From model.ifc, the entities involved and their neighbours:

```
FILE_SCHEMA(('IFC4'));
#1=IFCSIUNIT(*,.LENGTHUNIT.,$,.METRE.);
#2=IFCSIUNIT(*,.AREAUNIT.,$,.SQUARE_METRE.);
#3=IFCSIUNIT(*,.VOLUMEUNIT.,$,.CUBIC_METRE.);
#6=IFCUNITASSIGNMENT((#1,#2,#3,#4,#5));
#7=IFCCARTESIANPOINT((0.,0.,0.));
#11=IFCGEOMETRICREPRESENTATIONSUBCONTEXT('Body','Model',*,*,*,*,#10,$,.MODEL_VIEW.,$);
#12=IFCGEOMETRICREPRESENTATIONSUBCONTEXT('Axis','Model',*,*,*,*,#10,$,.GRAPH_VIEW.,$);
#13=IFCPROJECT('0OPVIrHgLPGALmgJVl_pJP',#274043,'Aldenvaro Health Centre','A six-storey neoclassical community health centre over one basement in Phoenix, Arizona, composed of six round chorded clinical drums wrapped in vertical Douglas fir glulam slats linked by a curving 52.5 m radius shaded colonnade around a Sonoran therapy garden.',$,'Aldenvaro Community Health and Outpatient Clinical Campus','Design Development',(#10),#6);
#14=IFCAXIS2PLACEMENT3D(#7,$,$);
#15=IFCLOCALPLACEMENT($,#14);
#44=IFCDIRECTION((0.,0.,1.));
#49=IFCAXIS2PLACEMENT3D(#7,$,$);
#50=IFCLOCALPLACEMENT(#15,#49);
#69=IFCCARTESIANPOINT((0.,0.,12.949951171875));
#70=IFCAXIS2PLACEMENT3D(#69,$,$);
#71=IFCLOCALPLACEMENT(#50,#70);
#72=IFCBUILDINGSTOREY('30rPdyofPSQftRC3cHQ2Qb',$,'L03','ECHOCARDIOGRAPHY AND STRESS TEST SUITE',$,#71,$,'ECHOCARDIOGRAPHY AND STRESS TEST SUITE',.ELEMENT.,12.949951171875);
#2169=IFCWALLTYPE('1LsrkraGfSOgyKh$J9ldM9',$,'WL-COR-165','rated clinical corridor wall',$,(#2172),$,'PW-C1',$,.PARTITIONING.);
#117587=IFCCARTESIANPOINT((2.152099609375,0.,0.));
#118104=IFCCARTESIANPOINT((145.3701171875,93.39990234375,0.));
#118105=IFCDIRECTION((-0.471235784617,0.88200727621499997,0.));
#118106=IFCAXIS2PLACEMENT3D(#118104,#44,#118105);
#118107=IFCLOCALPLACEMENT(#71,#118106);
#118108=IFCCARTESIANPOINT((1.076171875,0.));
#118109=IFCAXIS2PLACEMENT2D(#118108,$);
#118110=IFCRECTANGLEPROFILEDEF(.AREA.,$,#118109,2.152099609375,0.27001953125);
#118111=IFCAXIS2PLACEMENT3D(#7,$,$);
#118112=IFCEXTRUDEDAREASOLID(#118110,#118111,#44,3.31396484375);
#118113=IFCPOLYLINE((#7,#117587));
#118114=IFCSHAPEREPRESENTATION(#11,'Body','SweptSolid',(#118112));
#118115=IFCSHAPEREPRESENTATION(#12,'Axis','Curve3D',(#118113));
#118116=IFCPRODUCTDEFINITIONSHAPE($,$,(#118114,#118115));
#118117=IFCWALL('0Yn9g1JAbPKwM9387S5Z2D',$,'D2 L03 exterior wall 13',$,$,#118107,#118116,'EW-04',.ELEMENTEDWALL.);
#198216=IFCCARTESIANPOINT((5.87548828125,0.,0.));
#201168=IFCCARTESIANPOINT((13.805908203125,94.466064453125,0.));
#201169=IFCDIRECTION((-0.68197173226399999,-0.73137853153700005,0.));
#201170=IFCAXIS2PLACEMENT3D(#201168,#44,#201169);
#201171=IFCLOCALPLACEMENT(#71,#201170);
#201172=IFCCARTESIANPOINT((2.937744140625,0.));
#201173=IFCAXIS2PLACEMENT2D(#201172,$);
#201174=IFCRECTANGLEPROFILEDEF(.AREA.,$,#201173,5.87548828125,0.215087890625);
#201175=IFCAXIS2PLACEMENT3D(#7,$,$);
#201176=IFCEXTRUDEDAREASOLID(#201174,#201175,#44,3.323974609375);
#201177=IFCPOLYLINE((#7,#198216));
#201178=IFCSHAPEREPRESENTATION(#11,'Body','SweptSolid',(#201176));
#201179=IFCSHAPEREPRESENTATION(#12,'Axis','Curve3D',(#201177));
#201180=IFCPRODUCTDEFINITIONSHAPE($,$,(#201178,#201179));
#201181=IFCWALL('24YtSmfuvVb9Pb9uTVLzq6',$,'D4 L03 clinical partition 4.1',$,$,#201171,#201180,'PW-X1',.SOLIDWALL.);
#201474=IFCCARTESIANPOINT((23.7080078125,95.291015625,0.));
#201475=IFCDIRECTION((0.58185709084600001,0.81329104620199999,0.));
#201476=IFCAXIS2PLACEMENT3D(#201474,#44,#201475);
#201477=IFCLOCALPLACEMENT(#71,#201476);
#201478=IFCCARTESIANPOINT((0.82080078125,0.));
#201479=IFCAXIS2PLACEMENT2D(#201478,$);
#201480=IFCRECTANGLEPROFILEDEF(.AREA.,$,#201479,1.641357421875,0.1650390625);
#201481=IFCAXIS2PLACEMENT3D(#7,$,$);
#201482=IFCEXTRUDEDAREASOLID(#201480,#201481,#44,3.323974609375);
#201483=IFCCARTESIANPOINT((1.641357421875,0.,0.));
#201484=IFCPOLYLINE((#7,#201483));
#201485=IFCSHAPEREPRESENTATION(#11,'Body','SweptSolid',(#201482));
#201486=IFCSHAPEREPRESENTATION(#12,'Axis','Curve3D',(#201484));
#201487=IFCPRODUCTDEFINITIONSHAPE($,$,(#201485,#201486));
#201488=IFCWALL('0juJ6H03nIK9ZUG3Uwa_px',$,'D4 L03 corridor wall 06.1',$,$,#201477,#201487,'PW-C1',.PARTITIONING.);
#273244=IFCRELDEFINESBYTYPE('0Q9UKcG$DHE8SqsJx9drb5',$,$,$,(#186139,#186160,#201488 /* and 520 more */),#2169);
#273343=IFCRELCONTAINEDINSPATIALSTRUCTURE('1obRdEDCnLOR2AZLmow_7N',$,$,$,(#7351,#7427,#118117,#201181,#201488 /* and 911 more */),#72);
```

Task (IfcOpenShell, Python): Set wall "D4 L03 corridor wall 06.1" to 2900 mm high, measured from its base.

```python
import ifcopenshell
import ifcopenshell.geom
import ifcopenshell.util.representation
import ifcopenshell.util.shape
import ifcopenshell.util.unit

model = ifcopenshell.open("model.ifc")
unit_scale = ifcopenshell.util.unit.calculate_unit_scale(model)
settings = ifcopenshell.geom.settings()


def volume(element):
    """Net volume in cubic metres, openings subtracted."""
    shape = ifcopenshell.geom.create_shape(settings, element)
    return ifcopenshell.util.shape.get_volume(shape.geometry)


wall = model.by_guid("0juJ6H03nIK9ZUG3Uwa_px")
before = volume(wall)

body = ifcopenshell.util.representation.get_representation(wall, "Model", "Body")
solid = body.Items[0]
old_height = solid.Depth
solid.Depth = 2.9 / unit_scale
after = volume(wall)

print(f"height {old_height:g} -> {solid.Depth:g}, volume {before:.3f} -> {after:.3f} m3")

model.write("model_edited.ifc")
```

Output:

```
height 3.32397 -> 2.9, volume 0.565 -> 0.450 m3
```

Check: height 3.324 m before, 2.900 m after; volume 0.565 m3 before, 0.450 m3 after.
